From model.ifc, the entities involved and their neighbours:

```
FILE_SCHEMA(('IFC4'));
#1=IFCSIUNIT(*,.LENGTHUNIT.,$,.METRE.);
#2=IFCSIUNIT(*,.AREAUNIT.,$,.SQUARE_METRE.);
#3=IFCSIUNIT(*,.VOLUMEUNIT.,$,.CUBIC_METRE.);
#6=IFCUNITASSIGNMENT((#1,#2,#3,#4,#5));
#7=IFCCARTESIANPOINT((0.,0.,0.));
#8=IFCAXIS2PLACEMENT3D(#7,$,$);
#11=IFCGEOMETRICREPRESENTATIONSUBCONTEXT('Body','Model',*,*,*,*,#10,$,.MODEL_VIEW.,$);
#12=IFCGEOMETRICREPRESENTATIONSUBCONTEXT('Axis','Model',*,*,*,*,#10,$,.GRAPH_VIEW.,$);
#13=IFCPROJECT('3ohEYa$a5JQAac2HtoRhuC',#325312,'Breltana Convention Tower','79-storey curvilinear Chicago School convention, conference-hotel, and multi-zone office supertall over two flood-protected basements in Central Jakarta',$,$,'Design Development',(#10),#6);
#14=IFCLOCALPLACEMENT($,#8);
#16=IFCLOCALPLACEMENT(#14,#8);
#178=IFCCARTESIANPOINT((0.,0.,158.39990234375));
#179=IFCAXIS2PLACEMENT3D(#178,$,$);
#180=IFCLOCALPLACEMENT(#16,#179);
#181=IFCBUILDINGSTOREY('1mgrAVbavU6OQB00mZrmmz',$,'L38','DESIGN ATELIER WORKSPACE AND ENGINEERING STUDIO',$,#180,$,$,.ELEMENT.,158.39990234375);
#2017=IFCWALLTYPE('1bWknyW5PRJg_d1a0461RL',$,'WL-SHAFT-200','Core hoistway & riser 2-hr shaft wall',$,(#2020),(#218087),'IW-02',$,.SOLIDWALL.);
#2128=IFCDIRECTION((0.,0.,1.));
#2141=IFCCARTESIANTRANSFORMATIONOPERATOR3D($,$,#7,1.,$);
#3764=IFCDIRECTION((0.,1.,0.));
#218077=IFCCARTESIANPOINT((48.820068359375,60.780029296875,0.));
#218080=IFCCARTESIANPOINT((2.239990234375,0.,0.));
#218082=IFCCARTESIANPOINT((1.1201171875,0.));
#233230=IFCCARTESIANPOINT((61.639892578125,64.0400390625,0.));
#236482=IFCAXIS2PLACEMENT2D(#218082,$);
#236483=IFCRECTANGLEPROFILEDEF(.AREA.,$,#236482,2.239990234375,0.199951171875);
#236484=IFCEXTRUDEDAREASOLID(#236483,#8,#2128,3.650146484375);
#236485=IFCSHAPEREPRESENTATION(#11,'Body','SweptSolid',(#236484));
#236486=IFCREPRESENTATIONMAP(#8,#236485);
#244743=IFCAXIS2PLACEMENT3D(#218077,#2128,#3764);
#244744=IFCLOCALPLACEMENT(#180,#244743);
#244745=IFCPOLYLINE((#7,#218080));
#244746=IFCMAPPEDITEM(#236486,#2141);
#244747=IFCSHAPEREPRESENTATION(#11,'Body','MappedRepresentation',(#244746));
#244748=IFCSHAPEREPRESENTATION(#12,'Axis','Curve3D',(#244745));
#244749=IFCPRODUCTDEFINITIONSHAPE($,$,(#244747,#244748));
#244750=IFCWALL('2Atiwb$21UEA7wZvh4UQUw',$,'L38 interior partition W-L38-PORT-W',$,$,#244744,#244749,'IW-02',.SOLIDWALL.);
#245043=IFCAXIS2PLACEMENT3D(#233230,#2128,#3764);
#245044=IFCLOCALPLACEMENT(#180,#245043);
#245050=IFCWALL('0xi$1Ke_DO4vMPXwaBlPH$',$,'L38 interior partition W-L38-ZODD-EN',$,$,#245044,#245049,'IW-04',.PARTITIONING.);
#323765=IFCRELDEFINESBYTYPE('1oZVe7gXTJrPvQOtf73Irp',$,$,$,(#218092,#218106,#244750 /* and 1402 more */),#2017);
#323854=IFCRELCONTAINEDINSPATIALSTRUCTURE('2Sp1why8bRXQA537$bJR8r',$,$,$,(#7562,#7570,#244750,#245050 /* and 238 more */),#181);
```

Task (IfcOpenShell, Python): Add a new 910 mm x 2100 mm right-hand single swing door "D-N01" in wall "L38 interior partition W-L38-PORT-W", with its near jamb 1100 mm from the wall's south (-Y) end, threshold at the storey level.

```python
import numpy as np
import ifcopenshell
import ifcopenshell.api.feature
import ifcopenshell.api.geometry
import ifcopenshell.api.root
import ifcopenshell.api.spatial
import ifcopenshell.geom
import ifcopenshell.util.element
import ifcopenshell.util.placement
import ifcopenshell.util.representation
import ifcopenshell.util.shape
import ifcopenshell.util.unit

model = ifcopenshell.open("model.ifc")
unit_scale = ifcopenshell.util.unit.calculate_unit_scale(model)
settings = ifcopenshell.geom.settings()


def volume(element):
    """Net volume in cubic metres, openings subtracted."""
    shape = ifcopenshell.geom.create_shape(settings, element)
    return ifcopenshell.util.shape.get_volume(shape.geometry)


wall = model.by_id(244750)
storey = ifcopenshell.util.element.get_container(wall, ifc_class="IfcBuildingStorey")
context = ifcopenshell.util.representation.get_context(model, "Model", "Body", "MODEL_VIEW")
before = volume(wall)

width, height, from_end, sill = 0.91, 2.1, 1.1, 0.0  # metres

# The wall runs along its own X axis, and the end named is its -X end.
wall_shape = ifcopenshell.geom.create_shape(settings, wall)
x, y, z = ifcopenshell.util.shape.get_vertices(wall_shape.geometry).T
start = x.min() + from_end
face, thickness = float(y.min()), float(y.max() - y.min())
wall_matrix = ifcopenshell.util.placement.get_local_placement(wall.ObjectPlacement)
level = ifcopenshell.util.placement.get_local_placement(storey.ObjectPlacement)[2, 3]


def in_wall(x, y):
    """Placement at x, y metres in the wall's axes, at sill height."""
    matrix = wall_matrix.copy()
    matrix[:, 3] = wall_matrix @ np.array([x / unit_scale, y / unit_scale, 0.0, 1.0])
    matrix[2, 3] = level + sill / unit_scale
    return matrix


# Opening: a box that overshoots both wall faces by 50 mm.
opening = ifcopenshell.api.root.create_entity(model, ifc_class="IfcOpeningElement", predefined_type="OPENING")
box = ifcopenshell.api.geometry.add_wall_representation(
    model, context=context, length=width, height=height, thickness=thickness + 0.1
)
ifcopenshell.api.geometry.assign_representation(model, product=opening, representation=box)
ifcopenshell.api.geometry.edit_object_placement(model, product=opening, matrix=in_wall(start, face - 0.05), is_si=False)
ifcopenshell.api.feature.add_feature(model, feature=opening, element=wall)

door = ifcopenshell.api.root.create_entity(model, ifc_class="IfcDoor", name="D-N01", predefined_type="DOOR")
door.OverallWidth, door.OverallHeight = width / unit_scale, height / unit_scale
door.OperationType = "SINGLE_SWING_RIGHT"
body = ifcopenshell.api.geometry.add_door_representation(
    model,
    context=context,
    overall_width=door.OverallWidth,
    overall_height=door.OverallHeight,
    operation_type="SINGLE_SWING_RIGHT",
    lining_properties={"LiningDepth": thickness / unit_scale, "ThresholdDepth": thickness / unit_scale},
)
ifcopenshell.api.geometry.assign_representation(model, product=door, representation=body)
ifcopenshell.api.spatial.assign_container(model, products=[door], relating_structure=storey)
ifcopenshell.api.feature.add_filling(model, opening=opening, element=door)

# The lining spans the wall, so the door starts at the wall face.
ifcopenshell.api.geometry.edit_object_placement(model, product=door, matrix=in_wall(start, face), is_si=False)

after = volume(wall)

print(f"wall volume {before:.3f} -> {after:.3f} m3")

model.write("model-out.ifc")
```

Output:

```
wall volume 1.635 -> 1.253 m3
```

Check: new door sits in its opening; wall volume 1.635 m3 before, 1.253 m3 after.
